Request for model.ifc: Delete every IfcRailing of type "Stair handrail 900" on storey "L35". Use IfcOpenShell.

First a look at what the model holds.

```python
import ifcopenshell
import ifcopenshell.util.element

model = ifcopenshell.open("model.ifc")
print(model.schema)
storey = next(s for s in model.by_type("IfcBuildingStorey") if s.Name == "L35")
railings = [e for e in ifcopenshell.util.element.get_decomposition(storey) if e.is_a("IfcRailing")]
seen = {}
for e in railings:
    element_type = ifcopenshell.util.element.get_type(e)
    name = element_type.Name if element_type not in (None, e) else None
    seen[name] = seen.get(name, 0) + 1
for name, count in sorted(seen.items(), key=str):
    print(count, "x", name)
```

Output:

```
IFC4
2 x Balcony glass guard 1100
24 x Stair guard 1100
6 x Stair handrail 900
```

```python
import ifcopenshell
import ifcopenshell.api.root
import ifcopenshell.util.element

model = ifcopenshell.open("model.ifc")

storey = next(s for s in model.by_type("IfcBuildingStorey") if s.Name == "L35")
railings = [e for e in ifcopenshell.util.element.get_decomposition(storey) if e.is_a("IfcRailing")]
targets = [e for e in railings if (t := ifcopenshell.util.element.get_type(e)) not in (None, e) and t.Name == "Stair handrail 900"]

for e in targets:
    ifcopenshell.api.root.remove_product(model, product=e)
print(len(targets), "removed")

model.write("model_rev.ifc")
```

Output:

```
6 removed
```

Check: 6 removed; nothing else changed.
